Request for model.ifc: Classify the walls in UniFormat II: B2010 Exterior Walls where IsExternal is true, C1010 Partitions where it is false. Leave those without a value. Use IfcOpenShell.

First a look at what the model holds.

```python
import ifcopenshell
import ifcopenshell.util.element

model = ifcopenshell.open("model.ifc")
print(model.schema)
print("classifications:", [c.Name for c in model.by_type("IfcClassification")])
values = [ifcopenshell.util.element.get_pset(e, "Pset_WallCommon", "IsExternal") for e in model.by_type("IfcWall")]
for value in (True, False, None):
    print("IsExternal", value, values.count(value))
```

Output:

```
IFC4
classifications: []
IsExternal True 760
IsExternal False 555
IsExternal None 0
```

```python
import ifcopenshell
import ifcopenshell.api.classification
import ifcopenshell.util.element

model = ifcopenshell.open("model.ifc")

system = ifcopenshell.api.classification.add_classification(model, classification="UniFormat II")

walls = model.by_type("IfcWall")
external = {e: ifcopenshell.util.element.get_pset(e, "Pset_WallCommon", "IsExternal") for e in walls}
for flag, code, name in ((True, "B2010", "Exterior Walls"), (False, "C1010", "Partitions")):
    products = [e for e in walls if external[e] is flag]
    ifcopenshell.api.classification.add_reference(
        model, products=products, classification=system, identification=code, name=name
    )
    print(code, len(products))

model.write("model_edited.ifc")
```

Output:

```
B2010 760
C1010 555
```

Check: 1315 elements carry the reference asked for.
